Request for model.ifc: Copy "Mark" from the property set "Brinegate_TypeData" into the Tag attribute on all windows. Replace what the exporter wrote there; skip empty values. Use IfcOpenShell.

First a look at what the model holds.

```python
import ifcopenshell
import ifcopenshell.util.element

model = ifcopenshell.open("model.ifc")
print(model.schema)
windows = model.by_type("IfcWindow")
print(len(windows), "windows")
for e in windows[:8]:
    source = ifcopenshell.util.element.get_pset(e, "Brinegate_TypeData", "Mark")
    target = e.Tag
    print(e.id(), repr(source), repr(target), sep=" | ")
```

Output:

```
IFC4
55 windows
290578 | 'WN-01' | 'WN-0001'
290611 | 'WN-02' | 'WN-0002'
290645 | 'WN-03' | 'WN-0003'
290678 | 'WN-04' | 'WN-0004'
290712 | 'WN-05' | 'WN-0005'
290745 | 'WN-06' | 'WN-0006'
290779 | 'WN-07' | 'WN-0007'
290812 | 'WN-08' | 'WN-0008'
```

```python
import ifcopenshell
import ifcopenshell.util.element

model = ifcopenshell.open("model.ifc")

count = 0
for e in model.by_type("IfcWindow"):
    value = ifcopenshell.util.element.get_pset(e, "Brinegate_TypeData", "Mark")
    current = e.Tag
    if not value or not value.strip() or current == value:
        continue
    e.Tag = value
    count += 1

print(count, "windows updated")

model.write("model-out.ifc")
```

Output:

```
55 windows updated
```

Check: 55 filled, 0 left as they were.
